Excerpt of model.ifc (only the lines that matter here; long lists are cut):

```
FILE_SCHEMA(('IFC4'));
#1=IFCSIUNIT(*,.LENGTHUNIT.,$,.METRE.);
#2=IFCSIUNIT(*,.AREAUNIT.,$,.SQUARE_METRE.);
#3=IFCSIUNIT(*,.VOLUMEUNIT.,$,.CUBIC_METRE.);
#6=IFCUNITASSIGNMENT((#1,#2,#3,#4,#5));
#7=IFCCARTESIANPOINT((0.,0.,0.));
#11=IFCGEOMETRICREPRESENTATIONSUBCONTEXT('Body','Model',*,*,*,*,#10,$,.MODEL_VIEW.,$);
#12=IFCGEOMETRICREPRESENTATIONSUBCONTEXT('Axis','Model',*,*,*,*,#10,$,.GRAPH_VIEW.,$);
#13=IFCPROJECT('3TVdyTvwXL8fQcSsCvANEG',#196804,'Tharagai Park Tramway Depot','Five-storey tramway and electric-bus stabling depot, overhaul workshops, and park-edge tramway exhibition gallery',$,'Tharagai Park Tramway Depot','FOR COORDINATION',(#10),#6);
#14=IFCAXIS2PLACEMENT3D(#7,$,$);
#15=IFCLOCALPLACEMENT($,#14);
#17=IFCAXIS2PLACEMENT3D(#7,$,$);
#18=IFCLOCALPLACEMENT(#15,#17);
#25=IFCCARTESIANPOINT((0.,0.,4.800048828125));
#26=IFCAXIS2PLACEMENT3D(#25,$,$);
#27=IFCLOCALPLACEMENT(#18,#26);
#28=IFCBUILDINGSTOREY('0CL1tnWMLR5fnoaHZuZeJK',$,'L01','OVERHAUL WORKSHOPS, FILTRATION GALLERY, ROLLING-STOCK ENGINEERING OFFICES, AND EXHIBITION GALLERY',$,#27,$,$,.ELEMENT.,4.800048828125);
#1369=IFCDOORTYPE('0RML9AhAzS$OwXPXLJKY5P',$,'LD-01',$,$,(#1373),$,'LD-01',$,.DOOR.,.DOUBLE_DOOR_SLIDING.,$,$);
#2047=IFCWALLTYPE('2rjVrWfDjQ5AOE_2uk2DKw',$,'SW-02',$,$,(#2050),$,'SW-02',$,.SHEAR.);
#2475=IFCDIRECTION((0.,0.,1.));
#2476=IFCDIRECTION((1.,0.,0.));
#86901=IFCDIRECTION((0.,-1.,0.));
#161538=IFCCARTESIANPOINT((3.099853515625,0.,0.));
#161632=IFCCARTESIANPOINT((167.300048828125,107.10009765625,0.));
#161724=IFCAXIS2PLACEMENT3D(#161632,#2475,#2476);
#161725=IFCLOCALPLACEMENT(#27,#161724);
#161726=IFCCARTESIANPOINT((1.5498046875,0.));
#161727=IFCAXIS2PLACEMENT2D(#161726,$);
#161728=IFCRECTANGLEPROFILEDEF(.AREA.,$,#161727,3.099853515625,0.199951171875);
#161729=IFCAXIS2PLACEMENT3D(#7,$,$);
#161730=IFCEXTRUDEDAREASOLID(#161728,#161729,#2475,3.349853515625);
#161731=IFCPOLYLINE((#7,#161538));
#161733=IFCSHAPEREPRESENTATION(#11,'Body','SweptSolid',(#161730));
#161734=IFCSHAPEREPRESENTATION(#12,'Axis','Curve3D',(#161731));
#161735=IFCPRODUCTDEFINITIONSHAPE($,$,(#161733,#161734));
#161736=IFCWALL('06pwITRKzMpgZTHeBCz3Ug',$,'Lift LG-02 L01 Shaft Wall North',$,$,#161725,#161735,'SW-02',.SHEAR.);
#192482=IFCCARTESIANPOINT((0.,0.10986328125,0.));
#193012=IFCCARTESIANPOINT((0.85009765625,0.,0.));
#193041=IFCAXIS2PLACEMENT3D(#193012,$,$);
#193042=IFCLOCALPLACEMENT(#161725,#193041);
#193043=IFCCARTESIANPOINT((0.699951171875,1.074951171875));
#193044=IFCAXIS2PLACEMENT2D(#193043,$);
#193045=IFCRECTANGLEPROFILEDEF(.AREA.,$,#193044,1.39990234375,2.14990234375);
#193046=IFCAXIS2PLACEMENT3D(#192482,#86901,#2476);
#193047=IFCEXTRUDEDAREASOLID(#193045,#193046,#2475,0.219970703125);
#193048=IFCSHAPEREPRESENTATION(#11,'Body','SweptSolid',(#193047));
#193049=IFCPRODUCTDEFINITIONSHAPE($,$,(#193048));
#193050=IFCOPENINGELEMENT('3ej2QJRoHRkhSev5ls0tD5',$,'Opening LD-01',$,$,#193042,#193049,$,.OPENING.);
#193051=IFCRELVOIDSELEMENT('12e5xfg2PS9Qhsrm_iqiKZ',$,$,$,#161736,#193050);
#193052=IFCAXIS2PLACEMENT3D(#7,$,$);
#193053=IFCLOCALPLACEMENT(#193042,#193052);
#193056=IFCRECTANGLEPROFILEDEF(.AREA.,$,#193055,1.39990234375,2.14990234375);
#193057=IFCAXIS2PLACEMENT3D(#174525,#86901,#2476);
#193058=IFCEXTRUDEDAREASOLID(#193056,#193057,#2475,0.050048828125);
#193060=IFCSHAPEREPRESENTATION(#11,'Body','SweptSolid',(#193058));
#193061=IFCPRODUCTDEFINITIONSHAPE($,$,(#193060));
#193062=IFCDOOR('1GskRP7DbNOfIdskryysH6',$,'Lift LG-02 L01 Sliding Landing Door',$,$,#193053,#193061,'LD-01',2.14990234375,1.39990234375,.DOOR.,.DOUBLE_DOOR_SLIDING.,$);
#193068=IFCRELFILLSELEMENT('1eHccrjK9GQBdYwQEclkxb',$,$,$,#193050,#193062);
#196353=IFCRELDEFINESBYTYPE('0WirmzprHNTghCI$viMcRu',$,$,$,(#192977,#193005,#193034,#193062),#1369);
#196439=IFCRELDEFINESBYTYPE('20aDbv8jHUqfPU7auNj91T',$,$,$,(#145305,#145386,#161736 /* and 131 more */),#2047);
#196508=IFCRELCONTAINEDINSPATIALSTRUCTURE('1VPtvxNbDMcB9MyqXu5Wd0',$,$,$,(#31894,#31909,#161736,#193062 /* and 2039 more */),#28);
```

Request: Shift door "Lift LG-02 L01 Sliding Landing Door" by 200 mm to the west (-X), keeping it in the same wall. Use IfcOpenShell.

```python
import ifcopenshell
import ifcopenshell.api.geometry
import ifcopenshell.util.placement
import ifcopenshell.util.unit

model = ifcopenshell.open("model.ifc")
unit_scale = ifcopenshell.util.unit.calculate_unit_scale(model)

door = model.by_guid("1GskRP7DbNOfIdskryysH6")
opening = door.FillsVoids[0].RelatingOpeningElement
wall = opening.VoidsElements[0].RelatingBuildingElement

wall_matrix = ifcopenshell.util.placement.get_local_placement(wall.ObjectPlacement)
shift = wall_matrix[:3, 0] * -0.2 / unit_scale
before = ifcopenshell.util.placement.get_local_placement(door.ObjectPlacement)[:3, 3].copy()

# The door is placed relative to its opening, so it follows when the opening moves.
matrix = ifcopenshell.util.placement.get_local_placement(opening.ObjectPlacement)
matrix[:3, 3] += shift
ifcopenshell.api.geometry.edit_object_placement(
    model, product=opening, matrix=matrix, is_si=False, should_transform_children=True
)

after = ifcopenshell.util.placement.get_local_placement(door.ObjectPlacement)[:3, 3]
print("door moved by", (after - before).round(3) + 0.0)

model.write("model_rev.ifc")
```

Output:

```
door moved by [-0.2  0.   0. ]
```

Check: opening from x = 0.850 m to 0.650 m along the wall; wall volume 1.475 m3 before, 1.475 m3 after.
